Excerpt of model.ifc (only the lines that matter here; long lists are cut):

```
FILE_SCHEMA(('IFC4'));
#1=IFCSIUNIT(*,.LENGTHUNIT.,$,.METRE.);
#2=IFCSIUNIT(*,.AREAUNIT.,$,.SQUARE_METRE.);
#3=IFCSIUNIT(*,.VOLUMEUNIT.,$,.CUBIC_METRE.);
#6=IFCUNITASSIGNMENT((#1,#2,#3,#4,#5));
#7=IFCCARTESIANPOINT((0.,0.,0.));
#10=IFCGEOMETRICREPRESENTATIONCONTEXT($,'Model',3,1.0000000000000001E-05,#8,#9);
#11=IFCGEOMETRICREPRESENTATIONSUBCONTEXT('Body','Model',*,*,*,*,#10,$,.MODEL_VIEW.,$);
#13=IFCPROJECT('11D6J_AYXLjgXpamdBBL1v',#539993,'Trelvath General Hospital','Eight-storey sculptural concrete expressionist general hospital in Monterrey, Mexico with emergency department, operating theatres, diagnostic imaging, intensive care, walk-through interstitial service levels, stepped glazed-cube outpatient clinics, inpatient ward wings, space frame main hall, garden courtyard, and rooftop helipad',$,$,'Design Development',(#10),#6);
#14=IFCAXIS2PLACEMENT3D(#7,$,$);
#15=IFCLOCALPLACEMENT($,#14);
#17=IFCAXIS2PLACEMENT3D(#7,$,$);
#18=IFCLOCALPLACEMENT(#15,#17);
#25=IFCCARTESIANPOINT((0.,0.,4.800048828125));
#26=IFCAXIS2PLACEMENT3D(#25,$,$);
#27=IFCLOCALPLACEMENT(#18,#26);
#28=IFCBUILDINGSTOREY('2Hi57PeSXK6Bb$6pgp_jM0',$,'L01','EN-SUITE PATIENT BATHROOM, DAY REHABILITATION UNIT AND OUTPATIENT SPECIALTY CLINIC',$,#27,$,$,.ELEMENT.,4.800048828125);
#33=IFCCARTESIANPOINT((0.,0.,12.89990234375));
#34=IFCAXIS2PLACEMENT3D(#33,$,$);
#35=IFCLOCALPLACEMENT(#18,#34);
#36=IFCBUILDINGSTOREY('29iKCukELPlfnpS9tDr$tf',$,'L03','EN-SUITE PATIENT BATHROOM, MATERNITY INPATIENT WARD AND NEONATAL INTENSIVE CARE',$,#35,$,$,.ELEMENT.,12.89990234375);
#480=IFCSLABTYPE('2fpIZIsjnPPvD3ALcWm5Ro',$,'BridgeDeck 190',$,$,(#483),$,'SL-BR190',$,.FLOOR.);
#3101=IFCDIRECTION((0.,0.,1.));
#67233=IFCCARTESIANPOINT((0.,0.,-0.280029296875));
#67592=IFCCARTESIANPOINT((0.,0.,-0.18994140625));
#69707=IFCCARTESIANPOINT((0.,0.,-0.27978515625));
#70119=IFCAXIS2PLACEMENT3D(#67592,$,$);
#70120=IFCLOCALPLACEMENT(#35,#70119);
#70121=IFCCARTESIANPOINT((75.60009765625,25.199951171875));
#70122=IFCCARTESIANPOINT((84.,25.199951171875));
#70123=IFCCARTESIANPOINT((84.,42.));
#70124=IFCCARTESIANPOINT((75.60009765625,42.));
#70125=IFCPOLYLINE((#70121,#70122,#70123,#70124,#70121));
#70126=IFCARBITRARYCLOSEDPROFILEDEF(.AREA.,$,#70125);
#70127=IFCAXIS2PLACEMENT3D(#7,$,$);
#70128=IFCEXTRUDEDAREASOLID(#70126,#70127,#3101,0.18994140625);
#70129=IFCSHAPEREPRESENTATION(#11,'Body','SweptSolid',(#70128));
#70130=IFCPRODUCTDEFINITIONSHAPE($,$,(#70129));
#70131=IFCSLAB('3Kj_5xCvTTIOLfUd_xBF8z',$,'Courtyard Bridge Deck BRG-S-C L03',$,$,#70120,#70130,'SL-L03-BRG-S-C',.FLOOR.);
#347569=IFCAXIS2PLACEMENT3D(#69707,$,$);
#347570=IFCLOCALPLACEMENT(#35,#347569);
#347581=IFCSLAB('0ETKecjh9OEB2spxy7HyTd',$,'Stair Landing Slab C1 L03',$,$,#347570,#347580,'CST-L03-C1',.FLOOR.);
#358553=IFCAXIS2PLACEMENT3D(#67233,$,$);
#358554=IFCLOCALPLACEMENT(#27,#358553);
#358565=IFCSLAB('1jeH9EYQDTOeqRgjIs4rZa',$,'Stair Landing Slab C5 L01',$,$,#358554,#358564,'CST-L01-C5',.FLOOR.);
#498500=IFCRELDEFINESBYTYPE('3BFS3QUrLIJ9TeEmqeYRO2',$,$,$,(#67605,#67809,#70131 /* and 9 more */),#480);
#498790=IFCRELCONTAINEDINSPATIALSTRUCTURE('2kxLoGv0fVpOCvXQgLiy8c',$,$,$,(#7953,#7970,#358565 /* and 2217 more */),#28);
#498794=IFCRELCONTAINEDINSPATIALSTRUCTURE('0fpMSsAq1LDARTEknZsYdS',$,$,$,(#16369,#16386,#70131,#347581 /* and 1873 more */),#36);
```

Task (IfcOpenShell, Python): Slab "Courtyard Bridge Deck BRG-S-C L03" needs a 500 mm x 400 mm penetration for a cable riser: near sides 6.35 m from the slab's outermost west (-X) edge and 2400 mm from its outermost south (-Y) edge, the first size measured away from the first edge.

```python
import numpy as np
import ifcopenshell
import ifcopenshell.api.feature
import ifcopenshell.api.geometry
import ifcopenshell.api.root
import ifcopenshell.geom
import ifcopenshell.util.placement
import ifcopenshell.util.representation
import ifcopenshell.util.shape
import ifcopenshell.util.unit

model = ifcopenshell.open("model.ifc")
unit_scale = ifcopenshell.util.unit.calculate_unit_scale(model)
settings = ifcopenshell.geom.settings()


def volume(element):
    """Net volume in cubic metres, openings subtracted."""
    shape = ifcopenshell.geom.create_shape(settings, element)
    return ifcopenshell.util.shape.get_volume(shape.geometry)


slab = model.by_id(70131)
before = volume(slab)

# Extent in the slab's own axes, in metres. The edges named are its -X and -Y sides.
slab_shape = ifcopenshell.geom.create_shape(settings, slab)
vertices = ifcopenshell.util.shape.get_vertices(slab_shape.geometry)
x_min, y_min, bottom = vertices.min(axis=0)
top = vertices[:, 2].max()

opening = ifcopenshell.api.root.create_entity(model, ifc_class="IfcOpeningElement", name="Cable riser opening", predefined_type="OPENING")
context = ifcopenshell.util.representation.get_context(model, "Model", "Body", "MODEL_VIEW")
width, depth = 0.5, 0.4
outline = [(0.0, 0.0), (width, 0.0), (width, depth), (0.0, depth), (0.0, 0.0)]
# Overshoot both faces by 50 mm so the cut is clean.
shape = ifcopenshell.api.geometry.add_slab_representation(
    model, context=context, depth=top - bottom + 0.1, polyline=outline
)
ifcopenshell.api.geometry.assign_representation(model, product=opening, representation=shape)

matrix = ifcopenshell.util.placement.get_local_placement(slab.ObjectPlacement)
matrix[:, 3] = matrix @ np.append(np.array([x_min + 6.35, y_min + 2.4, bottom - 0.05]) / unit_scale, 1.0)
ifcopenshell.api.geometry.edit_object_placement(model, product=opening, matrix=matrix, is_si=False)
ifcopenshell.api.feature.add_feature(model, feature=opening, element=slab)

after = volume(slab)

print(f"slab volume {before:.3f} -> {after:.3f} m3")

model.write("model_updated.ifc")
```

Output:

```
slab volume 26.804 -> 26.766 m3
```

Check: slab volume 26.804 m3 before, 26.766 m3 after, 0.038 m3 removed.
